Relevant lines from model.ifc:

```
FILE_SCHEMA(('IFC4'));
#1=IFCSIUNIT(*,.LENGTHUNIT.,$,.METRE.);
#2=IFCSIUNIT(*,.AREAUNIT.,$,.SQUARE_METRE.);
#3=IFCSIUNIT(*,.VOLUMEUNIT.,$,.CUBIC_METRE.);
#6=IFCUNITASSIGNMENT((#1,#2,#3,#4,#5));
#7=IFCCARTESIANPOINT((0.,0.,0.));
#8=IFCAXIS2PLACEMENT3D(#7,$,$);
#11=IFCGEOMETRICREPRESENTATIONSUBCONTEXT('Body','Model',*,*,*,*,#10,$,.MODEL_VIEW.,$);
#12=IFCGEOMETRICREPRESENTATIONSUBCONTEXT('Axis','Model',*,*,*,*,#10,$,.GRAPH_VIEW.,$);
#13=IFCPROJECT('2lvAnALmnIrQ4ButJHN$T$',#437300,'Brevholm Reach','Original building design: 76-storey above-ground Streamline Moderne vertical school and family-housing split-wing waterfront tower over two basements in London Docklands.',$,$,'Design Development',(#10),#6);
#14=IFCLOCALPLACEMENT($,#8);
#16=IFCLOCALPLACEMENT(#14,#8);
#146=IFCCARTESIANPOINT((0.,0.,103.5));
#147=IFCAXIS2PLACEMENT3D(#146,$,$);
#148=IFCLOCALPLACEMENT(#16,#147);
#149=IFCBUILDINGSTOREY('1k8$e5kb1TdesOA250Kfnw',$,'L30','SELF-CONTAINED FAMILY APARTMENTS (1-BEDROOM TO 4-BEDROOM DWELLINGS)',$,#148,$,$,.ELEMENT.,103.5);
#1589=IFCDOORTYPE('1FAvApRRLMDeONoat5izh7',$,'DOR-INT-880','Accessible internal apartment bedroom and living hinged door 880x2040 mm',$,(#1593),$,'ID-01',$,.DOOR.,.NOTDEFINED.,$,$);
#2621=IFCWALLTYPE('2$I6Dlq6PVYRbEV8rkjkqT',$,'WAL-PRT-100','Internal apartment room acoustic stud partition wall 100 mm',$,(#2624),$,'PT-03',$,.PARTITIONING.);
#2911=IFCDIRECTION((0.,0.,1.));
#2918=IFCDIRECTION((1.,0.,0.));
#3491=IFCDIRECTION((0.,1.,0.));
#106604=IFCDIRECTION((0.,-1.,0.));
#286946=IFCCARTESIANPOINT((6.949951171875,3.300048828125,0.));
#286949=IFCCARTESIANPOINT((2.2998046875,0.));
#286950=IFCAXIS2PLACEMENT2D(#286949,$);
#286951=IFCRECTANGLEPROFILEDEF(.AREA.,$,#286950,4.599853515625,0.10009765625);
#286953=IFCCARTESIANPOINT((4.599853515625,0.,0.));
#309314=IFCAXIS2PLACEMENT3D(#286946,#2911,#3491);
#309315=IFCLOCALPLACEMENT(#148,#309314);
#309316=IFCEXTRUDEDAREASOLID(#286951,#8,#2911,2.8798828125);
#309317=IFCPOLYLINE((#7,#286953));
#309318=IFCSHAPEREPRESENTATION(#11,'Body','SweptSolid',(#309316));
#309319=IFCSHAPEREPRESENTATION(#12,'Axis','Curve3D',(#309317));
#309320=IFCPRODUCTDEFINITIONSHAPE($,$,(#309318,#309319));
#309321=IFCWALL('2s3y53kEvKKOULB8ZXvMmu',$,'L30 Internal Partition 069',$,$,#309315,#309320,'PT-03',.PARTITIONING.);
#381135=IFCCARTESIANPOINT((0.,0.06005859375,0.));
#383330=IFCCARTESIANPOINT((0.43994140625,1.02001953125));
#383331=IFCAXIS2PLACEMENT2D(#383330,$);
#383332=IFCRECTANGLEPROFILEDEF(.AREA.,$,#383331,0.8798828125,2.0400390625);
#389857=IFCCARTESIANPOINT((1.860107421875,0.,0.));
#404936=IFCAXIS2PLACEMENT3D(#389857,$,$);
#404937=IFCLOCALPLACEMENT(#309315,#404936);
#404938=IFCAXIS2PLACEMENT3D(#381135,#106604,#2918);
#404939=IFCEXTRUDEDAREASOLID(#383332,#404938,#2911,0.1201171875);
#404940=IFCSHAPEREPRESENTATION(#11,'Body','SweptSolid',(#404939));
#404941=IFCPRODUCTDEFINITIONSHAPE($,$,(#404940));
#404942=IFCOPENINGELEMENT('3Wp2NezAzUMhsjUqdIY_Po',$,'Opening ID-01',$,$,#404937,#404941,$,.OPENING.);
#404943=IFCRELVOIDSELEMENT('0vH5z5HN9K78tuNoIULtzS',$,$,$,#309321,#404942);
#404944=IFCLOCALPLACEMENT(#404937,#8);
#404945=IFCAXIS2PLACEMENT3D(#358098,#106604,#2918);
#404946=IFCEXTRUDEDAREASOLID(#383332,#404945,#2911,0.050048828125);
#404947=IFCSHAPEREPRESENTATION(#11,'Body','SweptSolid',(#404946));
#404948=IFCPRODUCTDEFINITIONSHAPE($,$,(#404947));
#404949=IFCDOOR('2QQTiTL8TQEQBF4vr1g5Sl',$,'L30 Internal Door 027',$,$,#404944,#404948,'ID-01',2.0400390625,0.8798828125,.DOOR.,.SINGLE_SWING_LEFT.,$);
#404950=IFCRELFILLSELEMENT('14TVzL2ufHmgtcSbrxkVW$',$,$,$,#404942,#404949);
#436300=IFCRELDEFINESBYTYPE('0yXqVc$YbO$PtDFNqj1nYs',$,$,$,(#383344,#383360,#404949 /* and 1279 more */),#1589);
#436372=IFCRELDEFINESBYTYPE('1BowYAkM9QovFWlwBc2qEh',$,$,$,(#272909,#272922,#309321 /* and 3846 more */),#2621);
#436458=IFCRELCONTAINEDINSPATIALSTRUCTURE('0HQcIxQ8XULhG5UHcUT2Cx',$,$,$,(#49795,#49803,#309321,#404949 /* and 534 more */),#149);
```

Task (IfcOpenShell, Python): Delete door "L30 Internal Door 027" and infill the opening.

```python
import ifcopenshell
import ifcopenshell.api.feature
import ifcopenshell.api.root
import ifcopenshell.geom
import ifcopenshell.util.shape

model = ifcopenshell.open("model.ifc")
settings = ifcopenshell.geom.settings()


def volume(element):
    """Net volume in cubic metres, openings subtracted."""
    shape = ifcopenshell.geom.create_shape(settings, element)
    return ifcopenshell.util.shape.get_volume(shape.geometry)


door = model.by_guid("2QQTiTL8TQEQBF4vr1g5Sl")
opening = door.FillsVoids[0].RelatingOpeningElement
wall = opening.VoidsElements[0].RelatingBuildingElement
before = volume(wall)

ifcopenshell.api.root.remove_product(model, product=door)
ifcopenshell.api.feature.remove_feature(model, feature=opening)

after = volume(wall)

print(f"wall volume {before:.3f} -> {after:.3f} m3")

model.write("model_updated.ifc")
```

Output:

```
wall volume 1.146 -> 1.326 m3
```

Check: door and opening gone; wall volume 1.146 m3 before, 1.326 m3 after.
